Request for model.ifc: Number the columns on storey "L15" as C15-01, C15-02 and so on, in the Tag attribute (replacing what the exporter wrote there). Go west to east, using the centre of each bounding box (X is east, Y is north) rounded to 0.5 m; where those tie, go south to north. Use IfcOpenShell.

First a look at what the model holds.

```python
import ifcopenshell
import ifcopenshell.util.element
import ifcopenshell.util.placement

model = ifcopenshell.open("model.ifc")
print(model.schema)
storey = next(s for s in model.by_type("IfcBuildingStorey") if s.Name == "L15")
columns = [e for e in ifcopenshell.util.element.get_decomposition(storey) if e.is_a("IfcColumn")]
for e in sorted(columns, key=lambda e: e.id()):
    origin = ifcopenshell.util.placement.get_local_placement(e.ObjectPlacement)[:3, 3]
    print(e.id(), e.Tag, e.Name, origin.round(2) + 0.0, sep=" | ")
```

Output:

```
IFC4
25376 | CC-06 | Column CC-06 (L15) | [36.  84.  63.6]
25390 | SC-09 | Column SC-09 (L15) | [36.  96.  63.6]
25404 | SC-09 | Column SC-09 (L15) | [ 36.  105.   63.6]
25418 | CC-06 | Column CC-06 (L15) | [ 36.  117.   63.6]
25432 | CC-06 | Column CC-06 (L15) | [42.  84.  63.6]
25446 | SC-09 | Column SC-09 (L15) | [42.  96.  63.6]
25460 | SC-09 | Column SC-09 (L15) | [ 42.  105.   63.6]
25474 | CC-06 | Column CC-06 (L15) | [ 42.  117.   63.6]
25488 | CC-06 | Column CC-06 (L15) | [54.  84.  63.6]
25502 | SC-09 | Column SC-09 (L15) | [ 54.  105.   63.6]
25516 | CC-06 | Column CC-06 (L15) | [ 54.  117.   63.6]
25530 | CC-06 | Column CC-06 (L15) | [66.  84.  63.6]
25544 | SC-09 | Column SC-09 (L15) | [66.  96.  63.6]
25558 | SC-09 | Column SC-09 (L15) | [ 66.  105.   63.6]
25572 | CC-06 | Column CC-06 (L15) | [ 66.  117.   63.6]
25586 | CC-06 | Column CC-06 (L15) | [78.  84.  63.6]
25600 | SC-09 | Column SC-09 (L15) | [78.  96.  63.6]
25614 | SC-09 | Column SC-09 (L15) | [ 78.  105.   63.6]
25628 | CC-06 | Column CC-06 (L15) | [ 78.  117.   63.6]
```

```python
import ifcopenshell
import ifcopenshell.geom
import ifcopenshell.util.element
import ifcopenshell.util.shape

model = ifcopenshell.open("model.ifc")
settings = ifcopenshell.geom.settings()
settings.set("use-world-coords", True)


def centre(element):
    shape = ifcopenshell.geom.create_shape(settings, element)
    return ifcopenshell.util.shape.get_bbox_centroid(shape.geometry)


storey = next(s for s in model.by_type("IfcBuildingStorey") if s.Name == "L15")
columns = [e for e in ifcopenshell.util.element.get_decomposition(storey) if e.is_a("IfcColumn")]

# Insertion points can sit at a corner or the storey origin, so sort by the geometry (in metres).
centres = {e: centre(e) for e in columns}
columns.sort(key=lambda e: (round(centres[e][0] / 0.5), centres[e][1]))

for i, e in enumerate(columns, start=1):
    number = f"C15-{i:02d}"
    e.Tag = number
    print(e.id(), number)

model.write("model-out.ifc")
```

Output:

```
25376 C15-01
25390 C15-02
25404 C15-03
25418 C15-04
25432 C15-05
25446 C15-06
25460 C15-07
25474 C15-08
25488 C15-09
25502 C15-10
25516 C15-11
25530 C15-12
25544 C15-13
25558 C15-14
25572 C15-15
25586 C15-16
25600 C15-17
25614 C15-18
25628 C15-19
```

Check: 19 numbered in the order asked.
